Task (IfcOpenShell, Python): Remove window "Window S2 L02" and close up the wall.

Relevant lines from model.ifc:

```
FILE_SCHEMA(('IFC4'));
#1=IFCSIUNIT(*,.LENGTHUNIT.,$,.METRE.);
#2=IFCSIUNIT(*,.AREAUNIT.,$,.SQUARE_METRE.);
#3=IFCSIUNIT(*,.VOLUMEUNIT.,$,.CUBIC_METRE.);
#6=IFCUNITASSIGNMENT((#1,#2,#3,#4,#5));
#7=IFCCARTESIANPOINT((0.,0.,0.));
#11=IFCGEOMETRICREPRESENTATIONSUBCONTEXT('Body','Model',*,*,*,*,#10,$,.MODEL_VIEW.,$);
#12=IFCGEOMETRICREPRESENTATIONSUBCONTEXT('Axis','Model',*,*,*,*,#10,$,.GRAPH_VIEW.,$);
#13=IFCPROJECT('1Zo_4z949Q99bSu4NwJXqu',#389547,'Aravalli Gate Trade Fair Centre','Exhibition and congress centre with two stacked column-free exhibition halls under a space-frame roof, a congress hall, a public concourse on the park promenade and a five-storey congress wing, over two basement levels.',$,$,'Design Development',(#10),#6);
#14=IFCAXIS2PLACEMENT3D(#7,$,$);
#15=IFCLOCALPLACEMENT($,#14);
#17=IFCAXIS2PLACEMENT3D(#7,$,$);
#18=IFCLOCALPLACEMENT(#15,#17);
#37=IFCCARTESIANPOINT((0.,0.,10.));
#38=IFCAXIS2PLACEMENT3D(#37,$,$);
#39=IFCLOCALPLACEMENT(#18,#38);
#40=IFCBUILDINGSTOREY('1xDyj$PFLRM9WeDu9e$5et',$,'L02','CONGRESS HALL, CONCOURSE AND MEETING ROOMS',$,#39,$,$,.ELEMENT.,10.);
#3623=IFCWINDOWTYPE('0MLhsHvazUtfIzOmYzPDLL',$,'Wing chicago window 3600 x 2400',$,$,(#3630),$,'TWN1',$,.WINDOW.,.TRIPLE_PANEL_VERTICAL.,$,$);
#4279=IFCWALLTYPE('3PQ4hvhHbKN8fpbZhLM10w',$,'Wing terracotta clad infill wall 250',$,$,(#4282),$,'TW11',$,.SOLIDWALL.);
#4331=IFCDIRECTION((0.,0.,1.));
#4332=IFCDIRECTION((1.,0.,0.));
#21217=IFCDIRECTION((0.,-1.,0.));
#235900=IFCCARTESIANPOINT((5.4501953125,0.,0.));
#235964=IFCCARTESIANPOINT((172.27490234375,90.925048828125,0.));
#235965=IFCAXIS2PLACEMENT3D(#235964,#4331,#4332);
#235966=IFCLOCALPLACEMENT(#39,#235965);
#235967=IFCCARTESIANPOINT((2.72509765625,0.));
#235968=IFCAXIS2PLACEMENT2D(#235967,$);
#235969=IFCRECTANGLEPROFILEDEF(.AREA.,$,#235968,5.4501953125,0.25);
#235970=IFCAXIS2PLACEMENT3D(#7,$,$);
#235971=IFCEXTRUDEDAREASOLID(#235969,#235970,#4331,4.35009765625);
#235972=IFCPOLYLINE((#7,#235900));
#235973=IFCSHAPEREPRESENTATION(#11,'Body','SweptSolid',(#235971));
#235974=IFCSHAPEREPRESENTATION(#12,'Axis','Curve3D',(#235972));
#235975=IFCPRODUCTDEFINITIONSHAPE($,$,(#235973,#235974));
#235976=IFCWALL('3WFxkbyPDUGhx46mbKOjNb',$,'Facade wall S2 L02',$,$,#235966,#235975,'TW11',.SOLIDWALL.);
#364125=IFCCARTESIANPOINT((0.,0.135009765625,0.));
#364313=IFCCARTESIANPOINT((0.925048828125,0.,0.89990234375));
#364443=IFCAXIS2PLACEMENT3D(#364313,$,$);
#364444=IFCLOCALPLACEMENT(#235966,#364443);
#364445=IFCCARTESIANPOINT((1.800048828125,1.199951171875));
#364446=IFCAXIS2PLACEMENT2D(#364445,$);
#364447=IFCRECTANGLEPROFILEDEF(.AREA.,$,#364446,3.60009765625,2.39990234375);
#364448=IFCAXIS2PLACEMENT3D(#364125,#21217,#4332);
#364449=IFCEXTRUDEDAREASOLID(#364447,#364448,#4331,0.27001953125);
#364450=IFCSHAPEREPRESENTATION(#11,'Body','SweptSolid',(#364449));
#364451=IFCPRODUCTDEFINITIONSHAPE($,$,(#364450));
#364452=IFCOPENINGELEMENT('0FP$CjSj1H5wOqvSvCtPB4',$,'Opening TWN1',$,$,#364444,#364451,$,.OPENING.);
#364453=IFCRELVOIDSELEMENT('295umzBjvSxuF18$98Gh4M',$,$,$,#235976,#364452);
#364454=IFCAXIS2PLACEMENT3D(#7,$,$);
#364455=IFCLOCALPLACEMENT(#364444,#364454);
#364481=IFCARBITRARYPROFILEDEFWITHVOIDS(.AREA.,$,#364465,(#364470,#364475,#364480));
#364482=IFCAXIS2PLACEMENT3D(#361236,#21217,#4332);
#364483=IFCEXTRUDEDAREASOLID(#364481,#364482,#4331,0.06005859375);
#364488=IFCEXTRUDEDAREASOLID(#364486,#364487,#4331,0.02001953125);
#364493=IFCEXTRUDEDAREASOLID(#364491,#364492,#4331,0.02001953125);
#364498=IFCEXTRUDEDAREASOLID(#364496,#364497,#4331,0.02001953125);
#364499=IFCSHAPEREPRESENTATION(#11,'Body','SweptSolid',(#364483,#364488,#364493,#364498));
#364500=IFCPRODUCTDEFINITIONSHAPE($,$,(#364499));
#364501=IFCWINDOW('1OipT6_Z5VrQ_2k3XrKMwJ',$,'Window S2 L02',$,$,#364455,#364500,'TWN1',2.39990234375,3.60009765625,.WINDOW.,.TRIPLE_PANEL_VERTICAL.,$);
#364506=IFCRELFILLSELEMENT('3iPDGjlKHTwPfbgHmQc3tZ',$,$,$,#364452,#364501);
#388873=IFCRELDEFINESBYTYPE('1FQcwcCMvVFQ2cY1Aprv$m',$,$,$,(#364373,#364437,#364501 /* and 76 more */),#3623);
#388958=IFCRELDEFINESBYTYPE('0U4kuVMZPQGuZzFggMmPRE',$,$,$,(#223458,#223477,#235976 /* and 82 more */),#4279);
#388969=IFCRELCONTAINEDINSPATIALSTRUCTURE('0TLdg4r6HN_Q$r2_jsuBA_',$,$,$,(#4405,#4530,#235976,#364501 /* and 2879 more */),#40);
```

```python
import ifcopenshell
import ifcopenshell.api.feature
import ifcopenshell.api.root
import ifcopenshell.geom
import ifcopenshell.util.shape

model = ifcopenshell.open("model.ifc")
settings = ifcopenshell.geom.settings()


def volume(element):
    """Net volume in cubic metres, openings subtracted."""
    shape = ifcopenshell.geom.create_shape(settings, element)
    return ifcopenshell.util.shape.get_volume(shape.geometry)


window = model.by_guid("1OipT6_Z5VrQ_2k3XrKMwJ")
opening = window.FillsVoids[0].RelatingOpeningElement
wall = opening.VoidsElements[0].RelatingBuildingElement
before = volume(wall)

ifcopenshell.api.root.remove_product(model, product=window)
ifcopenshell.api.feature.remove_feature(model, feature=opening)

after = volume(wall)

print(f"wall volume {before:.3f} -> {after:.3f} m3")

model.write("model-out.ifc")
```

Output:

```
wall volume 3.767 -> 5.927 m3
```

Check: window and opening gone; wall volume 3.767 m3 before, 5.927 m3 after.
